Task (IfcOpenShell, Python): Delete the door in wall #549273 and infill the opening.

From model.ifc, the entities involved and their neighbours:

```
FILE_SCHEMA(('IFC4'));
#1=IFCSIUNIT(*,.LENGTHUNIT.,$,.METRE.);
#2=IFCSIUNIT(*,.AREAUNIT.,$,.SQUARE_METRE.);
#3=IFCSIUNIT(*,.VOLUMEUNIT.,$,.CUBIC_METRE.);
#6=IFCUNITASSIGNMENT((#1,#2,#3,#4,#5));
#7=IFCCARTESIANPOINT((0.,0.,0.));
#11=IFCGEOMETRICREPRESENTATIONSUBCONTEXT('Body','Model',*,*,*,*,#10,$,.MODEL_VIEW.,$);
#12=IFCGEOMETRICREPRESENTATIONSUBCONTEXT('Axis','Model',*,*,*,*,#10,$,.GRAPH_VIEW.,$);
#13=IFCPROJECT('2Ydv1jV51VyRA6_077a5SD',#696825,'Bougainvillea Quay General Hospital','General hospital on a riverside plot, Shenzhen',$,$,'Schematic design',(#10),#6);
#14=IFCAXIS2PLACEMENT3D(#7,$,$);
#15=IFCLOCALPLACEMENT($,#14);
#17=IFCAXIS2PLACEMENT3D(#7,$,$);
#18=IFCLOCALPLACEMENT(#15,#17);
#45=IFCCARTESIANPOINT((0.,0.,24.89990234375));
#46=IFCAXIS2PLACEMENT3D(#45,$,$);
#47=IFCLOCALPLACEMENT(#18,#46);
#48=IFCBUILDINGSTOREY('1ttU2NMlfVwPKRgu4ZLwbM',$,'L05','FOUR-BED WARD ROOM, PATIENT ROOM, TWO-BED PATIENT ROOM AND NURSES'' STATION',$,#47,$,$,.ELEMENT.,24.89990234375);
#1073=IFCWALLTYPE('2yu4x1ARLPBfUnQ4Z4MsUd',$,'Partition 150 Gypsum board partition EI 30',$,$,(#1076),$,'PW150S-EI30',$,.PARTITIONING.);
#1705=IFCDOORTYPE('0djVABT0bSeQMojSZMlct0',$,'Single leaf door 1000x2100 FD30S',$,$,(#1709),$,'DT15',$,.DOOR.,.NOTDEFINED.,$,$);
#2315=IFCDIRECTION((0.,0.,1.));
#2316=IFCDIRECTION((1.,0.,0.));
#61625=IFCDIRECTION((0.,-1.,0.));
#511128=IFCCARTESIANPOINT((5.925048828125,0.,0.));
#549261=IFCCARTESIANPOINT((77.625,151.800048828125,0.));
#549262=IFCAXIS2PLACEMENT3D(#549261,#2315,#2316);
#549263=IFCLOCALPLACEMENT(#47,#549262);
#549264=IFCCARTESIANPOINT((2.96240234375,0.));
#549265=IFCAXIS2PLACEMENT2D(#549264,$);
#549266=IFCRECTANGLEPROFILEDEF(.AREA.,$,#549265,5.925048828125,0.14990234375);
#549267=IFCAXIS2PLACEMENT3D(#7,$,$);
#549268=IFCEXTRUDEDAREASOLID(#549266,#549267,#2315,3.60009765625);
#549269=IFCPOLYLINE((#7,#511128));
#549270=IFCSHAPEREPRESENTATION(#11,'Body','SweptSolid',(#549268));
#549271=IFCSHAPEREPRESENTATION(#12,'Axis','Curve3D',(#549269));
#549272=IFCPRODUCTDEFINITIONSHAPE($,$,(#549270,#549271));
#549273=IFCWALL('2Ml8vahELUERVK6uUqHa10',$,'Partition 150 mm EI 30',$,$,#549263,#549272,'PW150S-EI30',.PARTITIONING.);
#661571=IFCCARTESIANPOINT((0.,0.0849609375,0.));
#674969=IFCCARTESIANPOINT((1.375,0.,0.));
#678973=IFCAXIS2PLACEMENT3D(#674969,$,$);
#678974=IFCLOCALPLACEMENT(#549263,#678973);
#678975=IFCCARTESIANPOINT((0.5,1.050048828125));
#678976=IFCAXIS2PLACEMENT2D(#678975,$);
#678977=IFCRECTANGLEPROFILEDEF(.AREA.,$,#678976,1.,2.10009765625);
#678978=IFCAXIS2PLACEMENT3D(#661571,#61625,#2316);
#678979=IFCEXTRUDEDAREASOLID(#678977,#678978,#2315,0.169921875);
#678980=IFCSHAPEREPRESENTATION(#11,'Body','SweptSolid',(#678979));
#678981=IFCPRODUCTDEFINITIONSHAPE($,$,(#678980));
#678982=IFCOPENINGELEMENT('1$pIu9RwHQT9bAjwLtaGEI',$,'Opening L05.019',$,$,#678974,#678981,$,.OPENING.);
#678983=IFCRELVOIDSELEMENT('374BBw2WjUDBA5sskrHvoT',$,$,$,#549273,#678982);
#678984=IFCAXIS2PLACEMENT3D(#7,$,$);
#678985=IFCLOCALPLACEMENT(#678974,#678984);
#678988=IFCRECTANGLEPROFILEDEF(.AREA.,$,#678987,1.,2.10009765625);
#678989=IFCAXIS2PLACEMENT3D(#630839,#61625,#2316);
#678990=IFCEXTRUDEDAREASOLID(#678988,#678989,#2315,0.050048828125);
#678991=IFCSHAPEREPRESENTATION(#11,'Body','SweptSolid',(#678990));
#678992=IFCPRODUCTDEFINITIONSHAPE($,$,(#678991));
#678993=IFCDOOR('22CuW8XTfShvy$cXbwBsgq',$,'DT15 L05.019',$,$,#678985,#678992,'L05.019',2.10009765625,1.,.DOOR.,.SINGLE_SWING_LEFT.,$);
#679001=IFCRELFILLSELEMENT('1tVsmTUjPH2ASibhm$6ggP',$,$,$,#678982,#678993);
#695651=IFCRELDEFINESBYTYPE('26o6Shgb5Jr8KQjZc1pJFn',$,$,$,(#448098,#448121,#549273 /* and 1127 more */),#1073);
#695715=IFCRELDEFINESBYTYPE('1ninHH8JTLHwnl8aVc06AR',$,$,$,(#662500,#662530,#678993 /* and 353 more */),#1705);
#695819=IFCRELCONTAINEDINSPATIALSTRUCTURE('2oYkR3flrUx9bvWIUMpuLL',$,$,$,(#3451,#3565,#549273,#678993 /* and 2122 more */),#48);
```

```python
import ifcopenshell
import ifcopenshell.api.feature
import ifcopenshell.api.root
import ifcopenshell.geom
import ifcopenshell.util.shape

model = ifcopenshell.open("model.ifc")
settings = ifcopenshell.geom.settings()


def volume(element):
    """Net volume in cubic metres, openings subtracted."""
    shape = ifcopenshell.geom.create_shape(settings, element)
    return ifcopenshell.util.shape.get_volume(shape.geometry)


door = model.by_guid("22CuW8XTfShvy$cXbwBsgq")
opening = door.FillsVoids[0].RelatingOpeningElement
wall = opening.VoidsElements[0].RelatingBuildingElement
before = volume(wall)

ifcopenshell.api.root.remove_product(model, product=door)
ifcopenshell.api.feature.remove_feature(model, feature=opening)

after = volume(wall)

print(f"wall volume {before:.3f} -> {after:.3f} m3")

model.write("model_updated.ifc")
```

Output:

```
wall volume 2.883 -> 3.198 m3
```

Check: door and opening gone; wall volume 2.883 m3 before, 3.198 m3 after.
